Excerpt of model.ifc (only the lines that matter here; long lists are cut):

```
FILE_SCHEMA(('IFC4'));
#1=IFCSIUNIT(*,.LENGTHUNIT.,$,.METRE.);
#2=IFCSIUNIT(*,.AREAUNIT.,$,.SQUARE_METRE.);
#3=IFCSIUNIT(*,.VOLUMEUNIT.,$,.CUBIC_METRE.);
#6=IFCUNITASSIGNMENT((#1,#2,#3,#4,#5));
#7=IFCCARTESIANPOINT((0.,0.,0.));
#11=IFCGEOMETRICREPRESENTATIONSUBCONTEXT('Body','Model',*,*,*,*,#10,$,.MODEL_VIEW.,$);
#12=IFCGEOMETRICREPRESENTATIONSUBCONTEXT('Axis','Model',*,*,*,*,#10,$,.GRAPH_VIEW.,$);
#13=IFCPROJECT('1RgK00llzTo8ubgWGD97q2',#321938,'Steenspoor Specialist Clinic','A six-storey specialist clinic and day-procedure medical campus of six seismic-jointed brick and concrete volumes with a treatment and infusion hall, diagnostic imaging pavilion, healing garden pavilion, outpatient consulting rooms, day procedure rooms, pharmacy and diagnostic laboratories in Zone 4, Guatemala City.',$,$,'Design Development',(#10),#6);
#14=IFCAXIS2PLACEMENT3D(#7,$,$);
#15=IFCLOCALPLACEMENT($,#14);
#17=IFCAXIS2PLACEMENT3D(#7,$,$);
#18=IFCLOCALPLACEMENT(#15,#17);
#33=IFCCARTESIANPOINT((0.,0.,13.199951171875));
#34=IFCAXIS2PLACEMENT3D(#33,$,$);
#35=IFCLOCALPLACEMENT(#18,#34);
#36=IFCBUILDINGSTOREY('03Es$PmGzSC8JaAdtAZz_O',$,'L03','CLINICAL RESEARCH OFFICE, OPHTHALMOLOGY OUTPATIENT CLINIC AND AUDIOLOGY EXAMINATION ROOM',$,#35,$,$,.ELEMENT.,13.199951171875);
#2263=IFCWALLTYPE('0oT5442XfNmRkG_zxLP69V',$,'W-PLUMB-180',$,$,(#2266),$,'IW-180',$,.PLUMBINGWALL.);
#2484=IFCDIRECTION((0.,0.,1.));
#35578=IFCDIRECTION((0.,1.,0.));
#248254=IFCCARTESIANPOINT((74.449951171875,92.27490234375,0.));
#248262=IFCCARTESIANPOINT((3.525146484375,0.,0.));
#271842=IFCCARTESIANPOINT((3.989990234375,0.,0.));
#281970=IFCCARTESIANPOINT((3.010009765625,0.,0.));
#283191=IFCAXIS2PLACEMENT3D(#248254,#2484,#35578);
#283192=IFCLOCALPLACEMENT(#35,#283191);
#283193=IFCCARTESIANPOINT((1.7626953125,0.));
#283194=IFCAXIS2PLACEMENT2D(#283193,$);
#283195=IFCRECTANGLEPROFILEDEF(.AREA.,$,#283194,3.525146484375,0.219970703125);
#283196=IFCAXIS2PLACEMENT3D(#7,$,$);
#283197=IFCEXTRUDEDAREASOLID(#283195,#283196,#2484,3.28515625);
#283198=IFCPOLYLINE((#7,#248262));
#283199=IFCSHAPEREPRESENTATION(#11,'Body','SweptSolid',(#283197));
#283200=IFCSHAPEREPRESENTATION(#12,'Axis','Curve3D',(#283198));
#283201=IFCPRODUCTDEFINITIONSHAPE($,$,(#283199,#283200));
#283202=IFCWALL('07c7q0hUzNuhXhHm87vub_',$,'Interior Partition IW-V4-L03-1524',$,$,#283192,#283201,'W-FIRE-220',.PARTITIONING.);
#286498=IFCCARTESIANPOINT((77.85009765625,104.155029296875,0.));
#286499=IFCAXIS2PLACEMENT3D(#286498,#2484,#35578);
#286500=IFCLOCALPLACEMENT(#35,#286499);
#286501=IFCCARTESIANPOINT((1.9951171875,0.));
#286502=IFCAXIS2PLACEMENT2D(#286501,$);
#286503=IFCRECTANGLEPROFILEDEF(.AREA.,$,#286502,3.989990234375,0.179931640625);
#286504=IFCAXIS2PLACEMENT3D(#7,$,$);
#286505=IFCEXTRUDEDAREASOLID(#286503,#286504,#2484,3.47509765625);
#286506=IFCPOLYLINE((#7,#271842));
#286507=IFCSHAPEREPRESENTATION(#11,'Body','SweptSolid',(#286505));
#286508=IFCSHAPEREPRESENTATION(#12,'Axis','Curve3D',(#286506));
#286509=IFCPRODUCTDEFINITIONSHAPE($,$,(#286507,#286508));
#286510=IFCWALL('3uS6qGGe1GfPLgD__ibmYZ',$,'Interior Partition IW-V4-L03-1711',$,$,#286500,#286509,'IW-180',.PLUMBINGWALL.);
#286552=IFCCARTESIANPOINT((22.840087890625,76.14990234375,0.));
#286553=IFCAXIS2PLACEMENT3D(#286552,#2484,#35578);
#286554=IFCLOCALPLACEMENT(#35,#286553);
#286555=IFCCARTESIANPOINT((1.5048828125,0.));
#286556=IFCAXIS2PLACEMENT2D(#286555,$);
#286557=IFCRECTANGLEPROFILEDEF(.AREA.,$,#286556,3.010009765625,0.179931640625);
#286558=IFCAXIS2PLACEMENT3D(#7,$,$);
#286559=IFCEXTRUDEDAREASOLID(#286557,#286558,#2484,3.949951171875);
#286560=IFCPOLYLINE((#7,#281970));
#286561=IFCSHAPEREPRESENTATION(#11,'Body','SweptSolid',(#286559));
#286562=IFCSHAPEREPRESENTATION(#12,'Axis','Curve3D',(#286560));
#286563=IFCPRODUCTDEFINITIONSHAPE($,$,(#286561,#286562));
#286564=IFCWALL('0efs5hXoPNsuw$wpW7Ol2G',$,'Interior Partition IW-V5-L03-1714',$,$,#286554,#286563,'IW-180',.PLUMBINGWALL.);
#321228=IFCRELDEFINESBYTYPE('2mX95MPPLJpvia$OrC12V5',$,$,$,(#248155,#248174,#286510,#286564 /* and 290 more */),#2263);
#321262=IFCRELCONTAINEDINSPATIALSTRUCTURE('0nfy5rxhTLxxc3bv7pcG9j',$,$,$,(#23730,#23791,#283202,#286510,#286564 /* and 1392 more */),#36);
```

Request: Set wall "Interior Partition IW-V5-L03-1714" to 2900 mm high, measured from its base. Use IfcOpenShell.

```python
import ifcopenshell
import ifcopenshell.geom
import ifcopenshell.util.representation
import ifcopenshell.util.shape

model = ifcopenshell.open("model.ifc")
settings = ifcopenshell.geom.settings()


def volume(element):
    """Net volume in cubic metres, openings subtracted."""
    shape = ifcopenshell.geom.create_shape(settings, element)
    return ifcopenshell.util.shape.get_volume(shape.geometry)


wall = model.by_id(286564)
before = volume(wall)

body = ifcopenshell.util.representation.get_representation(wall, "Model", "Body")
solid = body.Items[0]
old_height = solid.Depth
solid.Depth = 2.9
after = volume(wall)

print(f"height {old_height:g} -> {solid.Depth:g}, volume {before:.3f} -> {after:.3f} m3")

model.write("model_rev.ifc")
```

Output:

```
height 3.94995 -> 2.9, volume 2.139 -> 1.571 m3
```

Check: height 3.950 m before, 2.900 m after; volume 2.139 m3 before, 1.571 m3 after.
